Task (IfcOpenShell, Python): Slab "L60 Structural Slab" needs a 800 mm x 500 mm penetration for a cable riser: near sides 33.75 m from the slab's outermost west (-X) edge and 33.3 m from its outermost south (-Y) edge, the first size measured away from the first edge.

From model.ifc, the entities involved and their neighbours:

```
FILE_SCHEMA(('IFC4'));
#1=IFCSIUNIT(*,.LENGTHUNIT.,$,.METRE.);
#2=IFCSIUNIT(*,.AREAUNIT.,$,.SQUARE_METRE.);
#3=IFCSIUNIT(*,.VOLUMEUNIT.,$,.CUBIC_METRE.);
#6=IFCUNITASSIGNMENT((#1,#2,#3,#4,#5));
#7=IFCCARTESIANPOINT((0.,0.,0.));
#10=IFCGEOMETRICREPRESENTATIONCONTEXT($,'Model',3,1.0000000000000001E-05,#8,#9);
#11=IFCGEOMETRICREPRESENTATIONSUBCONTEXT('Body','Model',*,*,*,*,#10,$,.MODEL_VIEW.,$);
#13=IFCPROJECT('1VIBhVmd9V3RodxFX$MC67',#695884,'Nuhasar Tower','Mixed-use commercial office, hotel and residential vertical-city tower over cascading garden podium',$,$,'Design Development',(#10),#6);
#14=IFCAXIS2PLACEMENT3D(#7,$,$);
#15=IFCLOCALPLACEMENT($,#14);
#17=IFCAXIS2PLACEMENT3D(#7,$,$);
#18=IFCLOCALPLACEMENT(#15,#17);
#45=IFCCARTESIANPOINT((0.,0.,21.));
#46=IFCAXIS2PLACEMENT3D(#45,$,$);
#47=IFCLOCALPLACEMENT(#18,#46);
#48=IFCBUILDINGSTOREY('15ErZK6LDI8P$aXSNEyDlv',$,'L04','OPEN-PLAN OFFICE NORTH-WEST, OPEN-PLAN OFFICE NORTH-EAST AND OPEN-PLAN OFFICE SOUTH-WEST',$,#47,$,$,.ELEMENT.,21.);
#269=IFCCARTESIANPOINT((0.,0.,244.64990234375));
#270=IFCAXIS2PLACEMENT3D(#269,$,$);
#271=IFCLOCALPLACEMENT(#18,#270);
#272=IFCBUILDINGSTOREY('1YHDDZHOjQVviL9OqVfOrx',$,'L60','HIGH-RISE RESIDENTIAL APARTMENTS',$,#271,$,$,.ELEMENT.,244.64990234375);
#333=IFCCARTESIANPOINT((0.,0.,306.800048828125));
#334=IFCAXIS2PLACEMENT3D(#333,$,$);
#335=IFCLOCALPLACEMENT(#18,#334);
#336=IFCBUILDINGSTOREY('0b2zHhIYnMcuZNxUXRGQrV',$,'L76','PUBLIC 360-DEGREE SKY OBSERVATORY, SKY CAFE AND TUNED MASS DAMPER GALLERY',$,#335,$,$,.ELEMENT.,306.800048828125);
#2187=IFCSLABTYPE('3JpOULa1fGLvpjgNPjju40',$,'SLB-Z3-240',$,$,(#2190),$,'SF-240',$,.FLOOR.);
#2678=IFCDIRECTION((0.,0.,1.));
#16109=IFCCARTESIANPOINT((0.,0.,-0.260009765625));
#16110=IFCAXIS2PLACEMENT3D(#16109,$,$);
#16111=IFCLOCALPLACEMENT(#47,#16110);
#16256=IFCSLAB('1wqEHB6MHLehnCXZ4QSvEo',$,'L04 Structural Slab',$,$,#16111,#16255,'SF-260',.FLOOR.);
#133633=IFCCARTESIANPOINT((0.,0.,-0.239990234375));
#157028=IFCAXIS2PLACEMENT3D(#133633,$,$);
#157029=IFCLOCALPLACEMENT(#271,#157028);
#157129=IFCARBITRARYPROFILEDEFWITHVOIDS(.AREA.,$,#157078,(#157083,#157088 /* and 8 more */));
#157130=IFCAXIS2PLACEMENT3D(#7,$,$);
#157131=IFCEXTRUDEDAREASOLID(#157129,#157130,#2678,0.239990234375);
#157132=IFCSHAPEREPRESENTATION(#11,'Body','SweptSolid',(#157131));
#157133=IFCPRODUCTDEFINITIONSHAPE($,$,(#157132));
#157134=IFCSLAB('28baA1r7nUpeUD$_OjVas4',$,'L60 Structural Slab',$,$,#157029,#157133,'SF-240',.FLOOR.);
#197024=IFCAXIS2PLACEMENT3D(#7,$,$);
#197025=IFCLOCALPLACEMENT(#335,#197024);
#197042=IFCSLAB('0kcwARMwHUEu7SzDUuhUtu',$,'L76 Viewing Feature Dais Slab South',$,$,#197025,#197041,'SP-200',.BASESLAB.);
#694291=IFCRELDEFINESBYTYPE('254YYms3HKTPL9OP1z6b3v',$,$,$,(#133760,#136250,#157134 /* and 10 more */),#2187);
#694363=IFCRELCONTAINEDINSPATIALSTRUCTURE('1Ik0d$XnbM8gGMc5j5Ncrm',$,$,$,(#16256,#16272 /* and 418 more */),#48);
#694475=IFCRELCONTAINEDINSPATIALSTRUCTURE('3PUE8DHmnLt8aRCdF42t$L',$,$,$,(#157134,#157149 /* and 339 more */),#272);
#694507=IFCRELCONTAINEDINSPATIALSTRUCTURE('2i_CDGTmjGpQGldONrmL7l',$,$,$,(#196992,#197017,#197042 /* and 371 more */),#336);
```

```python
import numpy as np
import ifcopenshell
import ifcopenshell.api.feature
import ifcopenshell.api.geometry
import ifcopenshell.api.root
import ifcopenshell.geom
import ifcopenshell.util.placement
import ifcopenshell.util.representation
import ifcopenshell.util.shape
import ifcopenshell.util.unit

model = ifcopenshell.open("model.ifc")
unit_scale = ifcopenshell.util.unit.calculate_unit_scale(model)
settings = ifcopenshell.geom.settings()


def volume(element):
    """Net volume in cubic metres, openings subtracted."""
    shape = ifcopenshell.geom.create_shape(settings, element)
    return ifcopenshell.util.shape.get_volume(shape.geometry)


slab = model.by_guid("28baA1r7nUpeUD$_OjVas4")
before = volume(slab)

# Extent in the slab's own axes, in metres. The edges named are its -X and -Y sides.
slab_shape = ifcopenshell.geom.create_shape(settings, slab)
vertices = ifcopenshell.util.shape.get_vertices(slab_shape.geometry)
x_min, y_min, bottom = vertices.min(axis=0)
top = vertices[:, 2].max()

opening = ifcopenshell.api.root.create_entity(model, ifc_class="IfcOpeningElement", name="Cable riser opening", predefined_type="OPENING")
context = ifcopenshell.util.representation.get_context(model, "Model", "Body", "MODEL_VIEW")
width, depth = 0.8, 0.5
outline = [(0.0, 0.0), (width, 0.0), (width, depth), (0.0, depth), (0.0, 0.0)]
# Overshoot both faces by 50 mm so the cut is clean.
shape = ifcopenshell.api.geometry.add_slab_representation(
    model, context=context, depth=top - bottom + 0.1, polyline=outline
)
ifcopenshell.api.geometry.assign_representation(model, product=opening, representation=shape)

matrix = ifcopenshell.util.placement.get_local_placement(slab.ObjectPlacement)
matrix[:, 3] = matrix @ np.append(np.array([x_min + 33.75, y_min + 33.3, bottom - 0.05]) / unit_scale, 1.0)
ifcopenshell.api.geometry.edit_object_placement(model, product=opening, matrix=matrix, is_si=False)
ifcopenshell.api.feature.add_feature(model, feature=opening, element=slab)

after = volume(slab)

print(f"slab volume {before:.3f} -> {after:.3f} m3")

model.write("model_rev.ifc")
```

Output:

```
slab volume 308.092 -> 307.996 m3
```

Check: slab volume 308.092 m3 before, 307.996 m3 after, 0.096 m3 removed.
